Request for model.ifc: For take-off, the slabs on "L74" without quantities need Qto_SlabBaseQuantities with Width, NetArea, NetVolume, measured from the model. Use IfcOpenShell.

First a look at what the model holds.

```python
import ifcopenshell
import ifcopenshell.util.element
import ifcopenshell.util.unit

model = ifcopenshell.open("model.ifc")
print(model.schema)
for unit_type in ("LENGTHUNIT", "AREAUNIT", "VOLUMEUNIT"):
    print(unit_type, ifcopenshell.util.unit.calculate_unit_scale(model, unit_type))
storey = next(s for s in model.by_type("IfcBuildingStorey") if s.Name == "L74")
slabs = [e for e in ifcopenshell.util.element.get_decomposition(storey) if e.is_a("IfcSlab")]
for e in sorted(slabs, key=lambda e: e.id()):
    print(e.id(), e.is_a(), e.Name, list(ifcopenshell.util.element.get_psets(e, qtos_only=True)), sep=" | ")
```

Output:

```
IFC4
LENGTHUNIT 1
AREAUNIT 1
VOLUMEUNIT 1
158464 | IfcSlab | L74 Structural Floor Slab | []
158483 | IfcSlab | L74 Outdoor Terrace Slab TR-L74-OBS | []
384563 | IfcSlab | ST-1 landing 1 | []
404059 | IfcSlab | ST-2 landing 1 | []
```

```python
import ifcopenshell
import ifcopenshell.api.pset
import ifcopenshell.geom
import ifcopenshell.util.element
import ifcopenshell.util.shape
import ifcopenshell.util.unit

model = ifcopenshell.open("model.ifc")
unit_scale = ifcopenshell.util.unit.calculate_unit_scale(model)
area_scale = ifcopenshell.util.unit.calculate_unit_scale(model, "AREAUNIT")
volume_scale = ifcopenshell.util.unit.calculate_unit_scale(model, "VOLUMEUNIT")
settings = ifcopenshell.geom.settings()

storey = next(s for s in model.by_type("IfcBuildingStorey") if s.Name == "L74")
slabs = [e for e in ifcopenshell.util.element.get_decomposition(storey) if e.is_a("IfcSlab")]

for e in sorted(slabs, key=lambda e: e.id()):
    if ifcopenshell.util.element.get_psets(e, qtos_only=True, should_inherit=False):
        continue
    # Geometry comes back in metres, in the element's own axes.
    shape = ifcopenshell.geom.create_shape(settings, e)
    values = {
        "Width": ifcopenshell.util.shape.get_z(shape.geometry) / unit_scale,
        "NetArea": ifcopenshell.util.shape.get_footprint_area(shape.geometry) / area_scale,
        "NetVolume": ifcopenshell.util.shape.get_volume(shape.geometry) / volume_scale,
    }
    qto = ifcopenshell.api.pset.add_qto(model, product=e, name="Qto_SlabBaseQuantities")
    ifcopenshell.api.pset.edit_qto(model, qto=qto, properties=values)
    print(e.id(), {k: round(v, 3) for k, v in values.items()})

model.write("model_v2.ifc")
```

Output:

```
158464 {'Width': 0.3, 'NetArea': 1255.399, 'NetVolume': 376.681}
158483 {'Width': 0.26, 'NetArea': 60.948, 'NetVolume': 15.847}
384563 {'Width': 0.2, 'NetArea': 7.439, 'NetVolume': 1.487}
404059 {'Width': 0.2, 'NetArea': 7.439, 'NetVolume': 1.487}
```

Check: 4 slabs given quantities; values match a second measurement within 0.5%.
